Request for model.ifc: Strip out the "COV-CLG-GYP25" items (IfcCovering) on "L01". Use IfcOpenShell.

First a look at what the model holds.

```python
import ifcopenshell
import ifcopenshell.util.element

model = ifcopenshell.open("model.ifc")
print(model.schema)
storey = next(s for s in model.by_type("IfcBuildingStorey") if s.Name == "L01")
coverings = [e for e in ifcopenshell.util.element.get_decomposition(storey) if e.is_a("IfcCovering")]
seen = {}
for e in coverings:
    element_type = ifcopenshell.util.element.get_type(e)
    name = element_type.Name if element_type not in (None, e) else None
    seen[name] = seen.get(name, 0) + 1
for name, count in sorted(seen.items(), key=str):
    print(count, "x", name)
```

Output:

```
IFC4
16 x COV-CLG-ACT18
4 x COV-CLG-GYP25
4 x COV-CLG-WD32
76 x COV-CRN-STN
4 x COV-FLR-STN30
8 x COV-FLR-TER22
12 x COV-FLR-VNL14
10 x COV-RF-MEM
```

```python
import ifcopenshell
import ifcopenshell.api.root
import ifcopenshell.util.element

model = ifcopenshell.open("model.ifc")

storey = next(s for s in model.by_type("IfcBuildingStorey") if s.Name == "L01")
coverings = [e for e in ifcopenshell.util.element.get_decomposition(storey) if e.is_a("IfcCovering")]
targets = [e for e in coverings if (t := ifcopenshell.util.element.get_type(e)) not in (None, e) and t.Name == "COV-CLG-GYP25"]

for e in targets:
    ifcopenshell.api.root.remove_product(model, product=e)
print(len(targets), "removed")

model.write("model_updated.ifc")
```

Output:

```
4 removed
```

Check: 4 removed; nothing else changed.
